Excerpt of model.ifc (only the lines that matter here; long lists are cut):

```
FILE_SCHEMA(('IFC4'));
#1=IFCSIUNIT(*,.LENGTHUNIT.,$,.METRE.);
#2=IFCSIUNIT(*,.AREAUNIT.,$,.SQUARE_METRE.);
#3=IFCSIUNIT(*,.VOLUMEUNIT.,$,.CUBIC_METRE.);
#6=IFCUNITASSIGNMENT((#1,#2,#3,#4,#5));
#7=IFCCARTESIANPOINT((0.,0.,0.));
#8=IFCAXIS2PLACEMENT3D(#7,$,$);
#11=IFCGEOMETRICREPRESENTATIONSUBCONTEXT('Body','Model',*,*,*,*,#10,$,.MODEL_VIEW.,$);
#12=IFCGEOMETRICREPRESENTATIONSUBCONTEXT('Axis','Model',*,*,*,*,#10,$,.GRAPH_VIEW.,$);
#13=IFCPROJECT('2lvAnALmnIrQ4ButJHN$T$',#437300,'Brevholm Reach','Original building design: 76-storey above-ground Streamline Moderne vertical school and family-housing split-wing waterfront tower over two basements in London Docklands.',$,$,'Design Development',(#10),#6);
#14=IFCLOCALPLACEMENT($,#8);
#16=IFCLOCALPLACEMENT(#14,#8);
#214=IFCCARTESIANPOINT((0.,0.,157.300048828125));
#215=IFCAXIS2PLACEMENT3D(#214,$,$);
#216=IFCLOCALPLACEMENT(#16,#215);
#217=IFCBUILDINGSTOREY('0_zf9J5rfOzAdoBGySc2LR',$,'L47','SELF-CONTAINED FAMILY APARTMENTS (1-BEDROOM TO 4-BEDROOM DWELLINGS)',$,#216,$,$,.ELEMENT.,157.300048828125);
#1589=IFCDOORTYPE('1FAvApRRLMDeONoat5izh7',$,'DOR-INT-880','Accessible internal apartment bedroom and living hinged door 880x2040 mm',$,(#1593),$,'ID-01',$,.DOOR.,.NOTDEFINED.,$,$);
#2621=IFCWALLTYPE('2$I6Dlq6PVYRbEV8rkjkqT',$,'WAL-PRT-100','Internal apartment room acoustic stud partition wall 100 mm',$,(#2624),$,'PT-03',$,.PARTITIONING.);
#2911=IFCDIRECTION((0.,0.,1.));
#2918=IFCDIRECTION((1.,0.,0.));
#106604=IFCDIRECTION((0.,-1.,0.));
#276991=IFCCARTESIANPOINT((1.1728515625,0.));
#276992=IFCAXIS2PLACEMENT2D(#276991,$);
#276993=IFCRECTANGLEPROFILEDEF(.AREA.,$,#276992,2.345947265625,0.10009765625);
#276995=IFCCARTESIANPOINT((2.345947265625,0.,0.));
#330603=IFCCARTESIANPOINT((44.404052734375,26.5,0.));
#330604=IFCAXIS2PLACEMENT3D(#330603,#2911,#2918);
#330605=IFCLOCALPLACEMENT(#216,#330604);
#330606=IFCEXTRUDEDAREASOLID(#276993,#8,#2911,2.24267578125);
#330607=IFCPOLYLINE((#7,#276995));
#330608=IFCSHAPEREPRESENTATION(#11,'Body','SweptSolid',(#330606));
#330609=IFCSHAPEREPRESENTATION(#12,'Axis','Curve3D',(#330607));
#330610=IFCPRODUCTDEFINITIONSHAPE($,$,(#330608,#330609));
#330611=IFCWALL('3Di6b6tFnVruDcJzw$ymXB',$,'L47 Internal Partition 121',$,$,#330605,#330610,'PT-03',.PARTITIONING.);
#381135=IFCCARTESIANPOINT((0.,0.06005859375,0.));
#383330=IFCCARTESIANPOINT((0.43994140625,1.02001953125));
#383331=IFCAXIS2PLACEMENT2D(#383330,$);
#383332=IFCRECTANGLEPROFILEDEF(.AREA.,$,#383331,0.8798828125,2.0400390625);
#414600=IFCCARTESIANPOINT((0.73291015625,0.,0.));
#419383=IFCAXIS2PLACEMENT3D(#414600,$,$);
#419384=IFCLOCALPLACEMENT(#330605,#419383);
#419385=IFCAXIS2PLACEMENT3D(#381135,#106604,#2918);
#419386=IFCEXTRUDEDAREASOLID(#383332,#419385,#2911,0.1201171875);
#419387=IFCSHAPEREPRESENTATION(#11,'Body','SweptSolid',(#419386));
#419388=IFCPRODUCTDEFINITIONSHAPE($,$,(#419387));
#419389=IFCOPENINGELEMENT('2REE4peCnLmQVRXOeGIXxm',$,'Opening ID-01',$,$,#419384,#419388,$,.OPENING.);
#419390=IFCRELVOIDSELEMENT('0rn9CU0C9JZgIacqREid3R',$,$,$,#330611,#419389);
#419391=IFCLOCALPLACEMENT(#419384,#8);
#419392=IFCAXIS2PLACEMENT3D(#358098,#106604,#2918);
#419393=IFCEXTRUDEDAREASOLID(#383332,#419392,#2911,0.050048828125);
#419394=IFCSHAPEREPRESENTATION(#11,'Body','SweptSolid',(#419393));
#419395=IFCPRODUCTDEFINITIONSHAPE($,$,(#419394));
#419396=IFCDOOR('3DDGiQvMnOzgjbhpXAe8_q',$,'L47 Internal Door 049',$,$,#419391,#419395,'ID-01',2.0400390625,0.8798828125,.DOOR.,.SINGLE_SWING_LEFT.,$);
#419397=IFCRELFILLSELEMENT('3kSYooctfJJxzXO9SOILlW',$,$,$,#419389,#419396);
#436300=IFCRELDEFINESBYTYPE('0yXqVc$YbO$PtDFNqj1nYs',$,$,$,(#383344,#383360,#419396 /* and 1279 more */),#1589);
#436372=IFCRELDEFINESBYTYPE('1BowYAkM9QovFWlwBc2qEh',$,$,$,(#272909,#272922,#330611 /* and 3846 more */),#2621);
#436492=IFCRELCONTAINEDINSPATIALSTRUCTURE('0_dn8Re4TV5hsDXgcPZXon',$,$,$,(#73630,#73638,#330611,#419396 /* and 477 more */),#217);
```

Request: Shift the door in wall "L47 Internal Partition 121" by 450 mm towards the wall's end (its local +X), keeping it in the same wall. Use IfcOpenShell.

```python
import ifcopenshell
import ifcopenshell.api.geometry
import ifcopenshell.util.placement
import ifcopenshell.util.unit

model = ifcopenshell.open("model.ifc")
unit_scale = ifcopenshell.util.unit.calculate_unit_scale(model)

door = model.by_guid("3DDGiQvMnOzgjbhpXAe8_q")
opening = door.FillsVoids[0].RelatingOpeningElement
wall = opening.VoidsElements[0].RelatingBuildingElement

wall_matrix = ifcopenshell.util.placement.get_local_placement(wall.ObjectPlacement)
shift = wall_matrix[:3, 0] * 0.45 / unit_scale
before = ifcopenshell.util.placement.get_local_placement(door.ObjectPlacement)[:3, 3].copy()

# The door is placed relative to its opening, so it follows when the opening moves.
matrix = ifcopenshell.util.placement.get_local_placement(opening.ObjectPlacement)
matrix[:3, 3] += shift
ifcopenshell.api.geometry.edit_object_placement(
    model, product=opening, matrix=matrix, is_si=False, should_transform_children=True
)

after = ifcopenshell.util.placement.get_local_placement(door.ObjectPlacement)[:3, 3]
print("door moved by", (after - before).round(3) + 0.0)

model.write("model-out.ifc")
```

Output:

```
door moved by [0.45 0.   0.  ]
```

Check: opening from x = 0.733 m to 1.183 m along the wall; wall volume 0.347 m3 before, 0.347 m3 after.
